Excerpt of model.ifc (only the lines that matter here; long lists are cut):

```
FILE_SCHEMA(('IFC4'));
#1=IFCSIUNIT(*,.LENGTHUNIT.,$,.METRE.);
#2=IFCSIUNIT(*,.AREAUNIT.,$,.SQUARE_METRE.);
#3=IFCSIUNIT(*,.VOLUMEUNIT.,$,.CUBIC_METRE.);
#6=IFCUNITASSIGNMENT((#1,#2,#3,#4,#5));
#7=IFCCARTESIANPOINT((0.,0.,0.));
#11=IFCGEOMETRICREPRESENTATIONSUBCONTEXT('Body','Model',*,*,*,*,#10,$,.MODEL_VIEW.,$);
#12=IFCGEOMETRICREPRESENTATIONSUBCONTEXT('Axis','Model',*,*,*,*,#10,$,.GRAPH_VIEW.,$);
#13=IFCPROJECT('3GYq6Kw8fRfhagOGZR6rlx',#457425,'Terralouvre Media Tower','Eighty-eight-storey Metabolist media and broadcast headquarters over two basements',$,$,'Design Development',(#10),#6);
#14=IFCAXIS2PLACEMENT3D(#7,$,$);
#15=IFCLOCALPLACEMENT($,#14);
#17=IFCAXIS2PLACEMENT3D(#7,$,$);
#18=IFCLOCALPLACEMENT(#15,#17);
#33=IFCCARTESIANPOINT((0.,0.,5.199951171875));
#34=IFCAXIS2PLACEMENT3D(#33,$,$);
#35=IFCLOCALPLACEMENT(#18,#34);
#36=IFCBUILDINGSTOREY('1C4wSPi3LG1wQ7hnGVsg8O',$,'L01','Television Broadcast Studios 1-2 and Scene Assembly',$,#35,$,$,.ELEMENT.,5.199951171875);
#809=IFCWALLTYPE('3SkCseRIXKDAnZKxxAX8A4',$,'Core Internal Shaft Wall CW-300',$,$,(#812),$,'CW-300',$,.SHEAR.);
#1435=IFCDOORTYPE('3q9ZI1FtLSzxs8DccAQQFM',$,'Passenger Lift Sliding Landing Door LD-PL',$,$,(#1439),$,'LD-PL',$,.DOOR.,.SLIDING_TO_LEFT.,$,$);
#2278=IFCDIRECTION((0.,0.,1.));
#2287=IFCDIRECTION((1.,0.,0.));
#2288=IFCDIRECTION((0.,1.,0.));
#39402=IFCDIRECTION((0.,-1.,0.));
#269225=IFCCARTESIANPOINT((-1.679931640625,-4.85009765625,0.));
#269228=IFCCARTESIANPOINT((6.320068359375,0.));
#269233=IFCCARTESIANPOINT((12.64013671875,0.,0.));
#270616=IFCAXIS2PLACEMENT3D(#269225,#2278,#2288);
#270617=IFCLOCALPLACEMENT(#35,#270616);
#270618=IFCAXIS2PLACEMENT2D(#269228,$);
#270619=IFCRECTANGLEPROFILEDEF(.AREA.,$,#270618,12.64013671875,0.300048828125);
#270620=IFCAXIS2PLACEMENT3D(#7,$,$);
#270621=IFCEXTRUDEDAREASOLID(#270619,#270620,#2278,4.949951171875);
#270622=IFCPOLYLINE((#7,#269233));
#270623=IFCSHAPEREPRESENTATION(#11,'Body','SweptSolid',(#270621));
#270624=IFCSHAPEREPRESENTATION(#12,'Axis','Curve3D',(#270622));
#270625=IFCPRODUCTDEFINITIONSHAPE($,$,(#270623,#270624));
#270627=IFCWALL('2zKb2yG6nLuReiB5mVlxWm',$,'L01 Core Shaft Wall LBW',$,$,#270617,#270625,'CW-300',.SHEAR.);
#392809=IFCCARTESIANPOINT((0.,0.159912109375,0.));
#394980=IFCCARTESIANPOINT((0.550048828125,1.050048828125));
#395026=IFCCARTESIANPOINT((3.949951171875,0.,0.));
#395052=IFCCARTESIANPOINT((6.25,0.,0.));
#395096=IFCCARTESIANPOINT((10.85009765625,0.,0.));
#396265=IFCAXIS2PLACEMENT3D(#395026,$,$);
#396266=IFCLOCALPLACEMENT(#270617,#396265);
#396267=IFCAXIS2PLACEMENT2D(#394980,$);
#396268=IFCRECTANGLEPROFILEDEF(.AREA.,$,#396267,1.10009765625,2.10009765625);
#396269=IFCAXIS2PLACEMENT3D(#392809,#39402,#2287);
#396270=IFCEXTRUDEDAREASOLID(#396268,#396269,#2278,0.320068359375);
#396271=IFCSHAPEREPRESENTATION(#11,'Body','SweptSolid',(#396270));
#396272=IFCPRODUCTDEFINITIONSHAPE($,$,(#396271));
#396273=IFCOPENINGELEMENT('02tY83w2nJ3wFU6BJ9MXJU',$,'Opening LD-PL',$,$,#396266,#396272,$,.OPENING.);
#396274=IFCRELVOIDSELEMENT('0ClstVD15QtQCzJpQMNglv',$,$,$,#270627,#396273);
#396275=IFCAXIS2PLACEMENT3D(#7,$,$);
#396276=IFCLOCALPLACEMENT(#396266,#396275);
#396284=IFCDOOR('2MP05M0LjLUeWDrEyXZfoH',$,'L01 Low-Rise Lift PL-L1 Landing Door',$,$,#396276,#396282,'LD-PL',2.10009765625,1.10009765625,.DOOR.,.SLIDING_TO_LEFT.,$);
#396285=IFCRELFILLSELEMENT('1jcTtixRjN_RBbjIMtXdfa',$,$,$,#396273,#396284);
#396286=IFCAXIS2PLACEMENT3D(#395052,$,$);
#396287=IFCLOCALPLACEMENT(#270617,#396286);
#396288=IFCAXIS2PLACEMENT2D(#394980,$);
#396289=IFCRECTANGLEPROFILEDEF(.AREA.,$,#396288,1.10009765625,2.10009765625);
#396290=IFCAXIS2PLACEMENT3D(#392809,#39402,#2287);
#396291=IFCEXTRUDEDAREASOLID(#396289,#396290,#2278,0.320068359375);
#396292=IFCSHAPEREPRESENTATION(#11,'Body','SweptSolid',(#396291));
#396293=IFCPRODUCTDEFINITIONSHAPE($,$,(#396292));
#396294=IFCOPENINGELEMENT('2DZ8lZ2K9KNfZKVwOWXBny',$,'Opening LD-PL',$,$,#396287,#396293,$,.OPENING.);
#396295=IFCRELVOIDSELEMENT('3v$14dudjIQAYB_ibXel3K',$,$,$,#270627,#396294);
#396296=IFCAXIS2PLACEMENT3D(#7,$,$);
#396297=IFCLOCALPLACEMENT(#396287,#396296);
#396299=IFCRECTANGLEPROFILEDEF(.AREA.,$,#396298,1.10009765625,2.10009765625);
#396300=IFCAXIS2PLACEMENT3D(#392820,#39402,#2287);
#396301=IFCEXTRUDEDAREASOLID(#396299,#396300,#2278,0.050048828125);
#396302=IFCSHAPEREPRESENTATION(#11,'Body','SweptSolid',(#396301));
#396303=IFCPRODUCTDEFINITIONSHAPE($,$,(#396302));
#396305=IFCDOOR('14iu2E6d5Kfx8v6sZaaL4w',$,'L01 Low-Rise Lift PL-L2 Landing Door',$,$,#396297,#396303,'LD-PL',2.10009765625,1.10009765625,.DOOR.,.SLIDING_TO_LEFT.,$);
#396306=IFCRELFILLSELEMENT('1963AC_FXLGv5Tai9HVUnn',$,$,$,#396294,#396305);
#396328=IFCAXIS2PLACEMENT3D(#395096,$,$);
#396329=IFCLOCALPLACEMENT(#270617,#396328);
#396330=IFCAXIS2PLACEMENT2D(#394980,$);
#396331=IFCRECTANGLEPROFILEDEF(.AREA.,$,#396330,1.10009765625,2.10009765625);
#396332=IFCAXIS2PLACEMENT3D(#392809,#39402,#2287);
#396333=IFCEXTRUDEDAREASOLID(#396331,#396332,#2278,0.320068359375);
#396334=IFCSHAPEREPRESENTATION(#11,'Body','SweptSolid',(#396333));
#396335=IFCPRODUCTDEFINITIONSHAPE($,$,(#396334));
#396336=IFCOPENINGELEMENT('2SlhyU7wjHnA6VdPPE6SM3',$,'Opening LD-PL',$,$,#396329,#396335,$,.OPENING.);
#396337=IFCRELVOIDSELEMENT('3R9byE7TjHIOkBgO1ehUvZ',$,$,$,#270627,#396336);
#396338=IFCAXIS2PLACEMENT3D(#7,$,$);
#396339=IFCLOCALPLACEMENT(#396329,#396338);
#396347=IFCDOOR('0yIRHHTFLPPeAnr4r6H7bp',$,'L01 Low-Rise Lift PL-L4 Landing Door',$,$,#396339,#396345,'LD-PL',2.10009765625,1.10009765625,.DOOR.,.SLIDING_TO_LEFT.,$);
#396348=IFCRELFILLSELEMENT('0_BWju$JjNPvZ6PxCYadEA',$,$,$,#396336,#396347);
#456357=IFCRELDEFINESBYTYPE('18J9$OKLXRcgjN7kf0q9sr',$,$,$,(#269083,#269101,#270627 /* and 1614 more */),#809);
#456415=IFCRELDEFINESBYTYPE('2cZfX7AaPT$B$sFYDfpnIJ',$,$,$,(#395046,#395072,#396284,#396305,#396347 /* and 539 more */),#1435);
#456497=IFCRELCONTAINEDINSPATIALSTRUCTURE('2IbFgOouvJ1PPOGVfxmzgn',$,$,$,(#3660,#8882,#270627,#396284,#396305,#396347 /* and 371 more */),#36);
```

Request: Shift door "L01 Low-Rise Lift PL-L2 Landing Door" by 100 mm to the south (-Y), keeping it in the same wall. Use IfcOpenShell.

```python
import ifcopenshell
import ifcopenshell.api.geometry
import ifcopenshell.util.placement
import ifcopenshell.util.unit

model = ifcopenshell.open("model.ifc")
unit_scale = ifcopenshell.util.unit.calculate_unit_scale(model)

door = model.by_guid("14iu2E6d5Kfx8v6sZaaL4w")
opening = door.FillsVoids[0].RelatingOpeningElement
wall = opening.VoidsElements[0].RelatingBuildingElement

wall_matrix = ifcopenshell.util.placement.get_local_placement(wall.ObjectPlacement)
shift = wall_matrix[:3, 0] * -0.1 / unit_scale
before = ifcopenshell.util.placement.get_local_placement(door.ObjectPlacement)[:3, 3].copy()

# The door is placed relative to its opening, so it follows when the opening moves.
matrix = ifcopenshell.util.placement.get_local_placement(opening.ObjectPlacement)
matrix[:3, 3] += shift
ifcopenshell.api.geometry.edit_object_placement(
    model, product=opening, matrix=matrix, is_si=False, should_transform_children=True
)

after = ifcopenshell.util.placement.get_local_placement(door.ObjectPlacement)[:3, 3]
print("door moved by", (after - before).round(3) + 0.0)

model.write("model_edited.ifc")
```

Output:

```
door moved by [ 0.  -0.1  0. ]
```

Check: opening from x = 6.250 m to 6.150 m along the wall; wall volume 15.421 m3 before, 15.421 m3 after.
